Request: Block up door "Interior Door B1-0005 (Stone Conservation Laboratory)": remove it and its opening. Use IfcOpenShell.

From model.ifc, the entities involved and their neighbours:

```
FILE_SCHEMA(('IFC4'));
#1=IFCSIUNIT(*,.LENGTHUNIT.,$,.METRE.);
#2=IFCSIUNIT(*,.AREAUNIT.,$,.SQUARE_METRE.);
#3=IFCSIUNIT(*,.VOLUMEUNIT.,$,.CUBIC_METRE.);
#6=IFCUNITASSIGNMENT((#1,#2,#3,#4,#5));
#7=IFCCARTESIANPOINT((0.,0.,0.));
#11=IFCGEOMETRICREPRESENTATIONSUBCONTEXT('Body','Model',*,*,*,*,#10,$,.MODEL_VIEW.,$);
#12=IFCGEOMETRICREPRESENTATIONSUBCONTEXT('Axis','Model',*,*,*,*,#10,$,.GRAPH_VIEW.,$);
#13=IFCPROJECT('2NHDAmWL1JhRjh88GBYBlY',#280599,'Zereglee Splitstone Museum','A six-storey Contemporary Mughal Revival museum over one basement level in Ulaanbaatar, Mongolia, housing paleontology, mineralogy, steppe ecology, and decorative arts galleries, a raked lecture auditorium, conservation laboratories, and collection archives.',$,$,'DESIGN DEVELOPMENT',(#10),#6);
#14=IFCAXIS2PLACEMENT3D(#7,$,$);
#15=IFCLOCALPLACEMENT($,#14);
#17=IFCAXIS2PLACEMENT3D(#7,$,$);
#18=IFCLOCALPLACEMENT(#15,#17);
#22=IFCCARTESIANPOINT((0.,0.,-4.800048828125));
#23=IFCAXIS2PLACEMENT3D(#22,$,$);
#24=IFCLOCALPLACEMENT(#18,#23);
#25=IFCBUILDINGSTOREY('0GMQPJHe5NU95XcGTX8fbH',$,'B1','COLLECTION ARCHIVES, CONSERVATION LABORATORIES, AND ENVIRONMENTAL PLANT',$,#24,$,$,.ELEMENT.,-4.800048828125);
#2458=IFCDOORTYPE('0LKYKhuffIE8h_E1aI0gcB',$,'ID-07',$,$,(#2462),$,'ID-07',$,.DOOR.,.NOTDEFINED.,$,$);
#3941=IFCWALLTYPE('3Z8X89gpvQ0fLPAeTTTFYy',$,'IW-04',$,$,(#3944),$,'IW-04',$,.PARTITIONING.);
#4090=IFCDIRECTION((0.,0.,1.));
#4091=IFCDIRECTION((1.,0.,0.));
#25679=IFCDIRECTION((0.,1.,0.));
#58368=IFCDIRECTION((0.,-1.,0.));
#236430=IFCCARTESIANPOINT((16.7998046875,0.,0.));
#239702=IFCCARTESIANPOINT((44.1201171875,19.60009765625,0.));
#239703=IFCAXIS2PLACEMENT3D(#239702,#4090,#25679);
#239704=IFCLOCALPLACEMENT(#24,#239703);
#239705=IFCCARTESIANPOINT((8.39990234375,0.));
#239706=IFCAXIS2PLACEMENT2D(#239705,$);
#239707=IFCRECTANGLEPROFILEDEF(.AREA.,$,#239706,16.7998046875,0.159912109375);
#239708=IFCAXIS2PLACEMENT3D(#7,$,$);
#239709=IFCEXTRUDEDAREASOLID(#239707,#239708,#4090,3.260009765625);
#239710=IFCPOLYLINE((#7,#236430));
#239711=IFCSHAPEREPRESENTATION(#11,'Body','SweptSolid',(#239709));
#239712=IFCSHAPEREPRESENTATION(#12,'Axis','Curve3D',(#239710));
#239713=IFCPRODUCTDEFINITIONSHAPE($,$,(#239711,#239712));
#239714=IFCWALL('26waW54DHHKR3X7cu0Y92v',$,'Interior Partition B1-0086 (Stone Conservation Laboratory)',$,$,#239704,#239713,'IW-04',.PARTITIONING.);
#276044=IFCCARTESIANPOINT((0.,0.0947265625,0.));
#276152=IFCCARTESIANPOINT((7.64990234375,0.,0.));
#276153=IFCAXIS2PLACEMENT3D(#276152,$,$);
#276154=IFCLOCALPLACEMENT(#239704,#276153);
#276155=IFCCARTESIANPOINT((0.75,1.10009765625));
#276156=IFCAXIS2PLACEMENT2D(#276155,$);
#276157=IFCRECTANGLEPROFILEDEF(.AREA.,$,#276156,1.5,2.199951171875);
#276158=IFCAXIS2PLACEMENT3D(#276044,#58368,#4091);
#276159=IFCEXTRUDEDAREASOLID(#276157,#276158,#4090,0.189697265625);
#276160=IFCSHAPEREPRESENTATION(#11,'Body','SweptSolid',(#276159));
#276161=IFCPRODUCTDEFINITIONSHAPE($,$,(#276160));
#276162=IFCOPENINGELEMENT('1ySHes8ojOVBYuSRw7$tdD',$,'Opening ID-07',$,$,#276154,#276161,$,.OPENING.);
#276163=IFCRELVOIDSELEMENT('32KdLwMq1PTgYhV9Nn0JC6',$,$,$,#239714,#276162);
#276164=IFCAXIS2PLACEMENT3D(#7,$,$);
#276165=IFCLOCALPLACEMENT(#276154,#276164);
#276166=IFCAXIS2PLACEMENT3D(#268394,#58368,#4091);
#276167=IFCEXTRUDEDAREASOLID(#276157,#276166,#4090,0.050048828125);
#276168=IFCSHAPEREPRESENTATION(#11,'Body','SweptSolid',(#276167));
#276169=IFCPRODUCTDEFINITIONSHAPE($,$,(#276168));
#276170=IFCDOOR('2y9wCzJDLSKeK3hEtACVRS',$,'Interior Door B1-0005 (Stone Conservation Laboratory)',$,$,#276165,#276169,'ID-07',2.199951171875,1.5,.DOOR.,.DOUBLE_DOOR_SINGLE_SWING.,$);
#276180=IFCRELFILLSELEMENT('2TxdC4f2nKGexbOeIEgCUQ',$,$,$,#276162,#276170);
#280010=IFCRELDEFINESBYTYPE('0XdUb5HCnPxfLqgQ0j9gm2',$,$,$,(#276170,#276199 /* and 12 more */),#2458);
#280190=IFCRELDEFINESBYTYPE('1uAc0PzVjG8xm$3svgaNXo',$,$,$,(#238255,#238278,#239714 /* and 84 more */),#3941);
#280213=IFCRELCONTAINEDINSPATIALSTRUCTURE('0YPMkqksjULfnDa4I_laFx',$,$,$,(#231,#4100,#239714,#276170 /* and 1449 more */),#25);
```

```python
import ifcopenshell
import ifcopenshell.api.feature
import ifcopenshell.api.root
import ifcopenshell.geom
import ifcopenshell.util.shape

model = ifcopenshell.open("model.ifc")
settings = ifcopenshell.geom.settings()


def volume(element):
    """Net volume in cubic metres, openings subtracted."""
    shape = ifcopenshell.geom.create_shape(settings, element)
    return ifcopenshell.util.shape.get_volume(shape.geometry)


door = model.by_guid("2y9wCzJDLSKeK3hEtACVRS")
opening = door.FillsVoids[0].RelatingOpeningElement
wall = opening.VoidsElements[0].RelatingBuildingElement
before = volume(wall)

ifcopenshell.api.root.remove_product(model, product=door)
ifcopenshell.api.feature.remove_feature(model, feature=opening)

after = volume(wall)

print(f"wall volume {before:.3f} -> {after:.3f} m3")

model.write("model_updated.ifc")
```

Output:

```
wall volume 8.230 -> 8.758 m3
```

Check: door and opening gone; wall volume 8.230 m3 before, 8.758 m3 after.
